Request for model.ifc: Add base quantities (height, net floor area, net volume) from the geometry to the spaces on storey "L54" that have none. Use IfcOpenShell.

First a look at what the model holds.

```python
import ifcopenshell
import ifcopenshell.util.element
import ifcopenshell.util.unit

model = ifcopenshell.open("model.ifc")
print(model.schema)
for unit_type in ("LENGTHUNIT", "AREAUNIT", "VOLUMEUNIT"):
    print(unit_type, ifcopenshell.util.unit.calculate_unit_scale(model, unit_type))
storey = next(s for s in model.by_type("IfcBuildingStorey") if s.Name == "L54")
spaces = [e for e in ifcopenshell.util.element.get_decomposition(storey) if e.is_a("IfcSpace")]
for e in sorted(spaces, key=lambda e: e.id()):
    print(e.id(), e.is_a(), e.Name, list(ifcopenshell.util.element.get_psets(e, qtos_only=True)), sep=" | ")
```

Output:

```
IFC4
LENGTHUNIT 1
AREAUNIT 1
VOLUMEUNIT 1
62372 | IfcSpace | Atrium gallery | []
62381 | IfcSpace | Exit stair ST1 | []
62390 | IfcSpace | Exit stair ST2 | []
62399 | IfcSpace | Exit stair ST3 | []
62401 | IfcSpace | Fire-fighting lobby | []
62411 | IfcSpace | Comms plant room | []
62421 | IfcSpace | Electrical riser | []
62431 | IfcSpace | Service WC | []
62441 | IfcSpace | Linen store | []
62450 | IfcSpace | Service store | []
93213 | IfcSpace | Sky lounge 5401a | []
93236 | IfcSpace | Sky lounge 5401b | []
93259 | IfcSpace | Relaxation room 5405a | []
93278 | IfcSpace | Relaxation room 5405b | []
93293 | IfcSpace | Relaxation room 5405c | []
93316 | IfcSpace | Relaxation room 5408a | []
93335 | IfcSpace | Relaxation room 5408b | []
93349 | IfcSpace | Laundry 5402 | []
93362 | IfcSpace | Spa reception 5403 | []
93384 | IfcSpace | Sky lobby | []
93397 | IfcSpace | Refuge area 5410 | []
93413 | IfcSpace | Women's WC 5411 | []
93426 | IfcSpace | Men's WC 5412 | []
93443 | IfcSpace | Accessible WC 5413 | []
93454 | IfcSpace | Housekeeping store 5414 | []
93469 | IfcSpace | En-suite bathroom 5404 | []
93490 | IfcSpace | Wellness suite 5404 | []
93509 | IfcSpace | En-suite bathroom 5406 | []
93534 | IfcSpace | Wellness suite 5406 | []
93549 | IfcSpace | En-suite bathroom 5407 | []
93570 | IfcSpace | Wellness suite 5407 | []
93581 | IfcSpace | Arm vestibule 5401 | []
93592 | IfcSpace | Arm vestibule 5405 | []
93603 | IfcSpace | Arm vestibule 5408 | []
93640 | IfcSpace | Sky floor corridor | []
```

```python
import ifcopenshell
import ifcopenshell.api.pset
import ifcopenshell.geom
import ifcopenshell.util.element
import ifcopenshell.util.shape
import ifcopenshell.util.unit

model = ifcopenshell.open("model.ifc")
unit_scale = ifcopenshell.util.unit.calculate_unit_scale(model)
area_scale = ifcopenshell.util.unit.calculate_unit_scale(model, "AREAUNIT")
volume_scale = ifcopenshell.util.unit.calculate_unit_scale(model, "VOLUMEUNIT")
settings = ifcopenshell.geom.settings()

storey = next(s for s in model.by_type("IfcBuildingStorey") if s.Name == "L54")
spaces = [e for e in ifcopenshell.util.element.get_decomposition(storey) if e.is_a("IfcSpace")]

for e in sorted(spaces, key=lambda e: e.id()):
    if ifcopenshell.util.element.get_psets(e, qtos_only=True, should_inherit=False):
        continue
    # Geometry comes back in metres, in the element's own axes.
    shape = ifcopenshell.geom.create_shape(settings, e)
    values = {
        "Height": ifcopenshell.util.shape.get_z(shape.geometry) / unit_scale,
        "NetFloorArea": ifcopenshell.util.shape.get_footprint_area(shape.geometry) / area_scale,
        "NetVolume": ifcopenshell.util.shape.get_volume(shape.geometry) / volume_scale,
    }
    qto = ifcopenshell.api.pset.add_qto(model, product=e, name="Qto_SpaceBaseQuantities")
    ifcopenshell.api.pset.edit_qto(model, qto=qto, properties=values)
    print(e.id(), {k: round(v, 3) for k, v in values.items()})

model.write("model_edited.ifc")
```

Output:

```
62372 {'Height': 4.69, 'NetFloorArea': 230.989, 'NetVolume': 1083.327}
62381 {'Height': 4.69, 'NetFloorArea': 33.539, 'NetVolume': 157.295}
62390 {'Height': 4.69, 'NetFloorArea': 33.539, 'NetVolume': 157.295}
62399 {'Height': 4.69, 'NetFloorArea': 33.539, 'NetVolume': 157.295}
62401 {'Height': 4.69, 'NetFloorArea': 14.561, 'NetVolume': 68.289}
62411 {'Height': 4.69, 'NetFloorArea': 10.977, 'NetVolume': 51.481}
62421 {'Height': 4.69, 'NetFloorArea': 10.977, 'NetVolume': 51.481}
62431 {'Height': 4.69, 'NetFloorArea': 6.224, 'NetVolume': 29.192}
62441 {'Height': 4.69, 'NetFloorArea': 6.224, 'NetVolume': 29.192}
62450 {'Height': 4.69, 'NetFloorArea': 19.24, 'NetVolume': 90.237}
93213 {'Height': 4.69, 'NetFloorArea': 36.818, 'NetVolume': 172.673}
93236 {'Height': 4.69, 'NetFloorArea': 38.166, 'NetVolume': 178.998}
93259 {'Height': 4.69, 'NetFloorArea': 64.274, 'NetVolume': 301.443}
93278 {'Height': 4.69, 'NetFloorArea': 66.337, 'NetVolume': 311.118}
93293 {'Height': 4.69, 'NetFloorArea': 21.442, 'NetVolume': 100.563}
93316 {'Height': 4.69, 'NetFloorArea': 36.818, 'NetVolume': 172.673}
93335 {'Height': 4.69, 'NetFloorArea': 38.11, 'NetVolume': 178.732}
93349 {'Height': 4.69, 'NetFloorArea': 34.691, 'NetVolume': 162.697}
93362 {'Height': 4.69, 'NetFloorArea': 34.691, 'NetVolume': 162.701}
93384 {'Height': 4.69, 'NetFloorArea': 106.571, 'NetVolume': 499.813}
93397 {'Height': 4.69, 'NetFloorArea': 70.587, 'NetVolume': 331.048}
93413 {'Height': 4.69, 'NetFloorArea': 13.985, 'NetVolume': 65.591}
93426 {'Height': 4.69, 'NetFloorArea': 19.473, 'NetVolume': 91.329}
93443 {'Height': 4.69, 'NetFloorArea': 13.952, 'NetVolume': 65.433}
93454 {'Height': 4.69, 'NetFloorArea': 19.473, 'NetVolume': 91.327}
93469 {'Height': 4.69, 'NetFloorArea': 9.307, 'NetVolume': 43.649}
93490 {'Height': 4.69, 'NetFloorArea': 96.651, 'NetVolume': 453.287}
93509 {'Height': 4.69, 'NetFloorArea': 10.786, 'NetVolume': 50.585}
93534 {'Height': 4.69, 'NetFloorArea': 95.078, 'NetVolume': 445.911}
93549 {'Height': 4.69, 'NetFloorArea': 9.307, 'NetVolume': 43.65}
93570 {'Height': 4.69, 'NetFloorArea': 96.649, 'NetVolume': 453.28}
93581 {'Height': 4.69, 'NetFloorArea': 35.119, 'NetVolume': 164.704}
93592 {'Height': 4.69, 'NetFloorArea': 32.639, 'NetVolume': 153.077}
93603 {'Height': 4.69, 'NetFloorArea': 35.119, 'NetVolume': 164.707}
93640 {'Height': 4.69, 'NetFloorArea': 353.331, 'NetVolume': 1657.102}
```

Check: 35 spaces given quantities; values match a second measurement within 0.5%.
